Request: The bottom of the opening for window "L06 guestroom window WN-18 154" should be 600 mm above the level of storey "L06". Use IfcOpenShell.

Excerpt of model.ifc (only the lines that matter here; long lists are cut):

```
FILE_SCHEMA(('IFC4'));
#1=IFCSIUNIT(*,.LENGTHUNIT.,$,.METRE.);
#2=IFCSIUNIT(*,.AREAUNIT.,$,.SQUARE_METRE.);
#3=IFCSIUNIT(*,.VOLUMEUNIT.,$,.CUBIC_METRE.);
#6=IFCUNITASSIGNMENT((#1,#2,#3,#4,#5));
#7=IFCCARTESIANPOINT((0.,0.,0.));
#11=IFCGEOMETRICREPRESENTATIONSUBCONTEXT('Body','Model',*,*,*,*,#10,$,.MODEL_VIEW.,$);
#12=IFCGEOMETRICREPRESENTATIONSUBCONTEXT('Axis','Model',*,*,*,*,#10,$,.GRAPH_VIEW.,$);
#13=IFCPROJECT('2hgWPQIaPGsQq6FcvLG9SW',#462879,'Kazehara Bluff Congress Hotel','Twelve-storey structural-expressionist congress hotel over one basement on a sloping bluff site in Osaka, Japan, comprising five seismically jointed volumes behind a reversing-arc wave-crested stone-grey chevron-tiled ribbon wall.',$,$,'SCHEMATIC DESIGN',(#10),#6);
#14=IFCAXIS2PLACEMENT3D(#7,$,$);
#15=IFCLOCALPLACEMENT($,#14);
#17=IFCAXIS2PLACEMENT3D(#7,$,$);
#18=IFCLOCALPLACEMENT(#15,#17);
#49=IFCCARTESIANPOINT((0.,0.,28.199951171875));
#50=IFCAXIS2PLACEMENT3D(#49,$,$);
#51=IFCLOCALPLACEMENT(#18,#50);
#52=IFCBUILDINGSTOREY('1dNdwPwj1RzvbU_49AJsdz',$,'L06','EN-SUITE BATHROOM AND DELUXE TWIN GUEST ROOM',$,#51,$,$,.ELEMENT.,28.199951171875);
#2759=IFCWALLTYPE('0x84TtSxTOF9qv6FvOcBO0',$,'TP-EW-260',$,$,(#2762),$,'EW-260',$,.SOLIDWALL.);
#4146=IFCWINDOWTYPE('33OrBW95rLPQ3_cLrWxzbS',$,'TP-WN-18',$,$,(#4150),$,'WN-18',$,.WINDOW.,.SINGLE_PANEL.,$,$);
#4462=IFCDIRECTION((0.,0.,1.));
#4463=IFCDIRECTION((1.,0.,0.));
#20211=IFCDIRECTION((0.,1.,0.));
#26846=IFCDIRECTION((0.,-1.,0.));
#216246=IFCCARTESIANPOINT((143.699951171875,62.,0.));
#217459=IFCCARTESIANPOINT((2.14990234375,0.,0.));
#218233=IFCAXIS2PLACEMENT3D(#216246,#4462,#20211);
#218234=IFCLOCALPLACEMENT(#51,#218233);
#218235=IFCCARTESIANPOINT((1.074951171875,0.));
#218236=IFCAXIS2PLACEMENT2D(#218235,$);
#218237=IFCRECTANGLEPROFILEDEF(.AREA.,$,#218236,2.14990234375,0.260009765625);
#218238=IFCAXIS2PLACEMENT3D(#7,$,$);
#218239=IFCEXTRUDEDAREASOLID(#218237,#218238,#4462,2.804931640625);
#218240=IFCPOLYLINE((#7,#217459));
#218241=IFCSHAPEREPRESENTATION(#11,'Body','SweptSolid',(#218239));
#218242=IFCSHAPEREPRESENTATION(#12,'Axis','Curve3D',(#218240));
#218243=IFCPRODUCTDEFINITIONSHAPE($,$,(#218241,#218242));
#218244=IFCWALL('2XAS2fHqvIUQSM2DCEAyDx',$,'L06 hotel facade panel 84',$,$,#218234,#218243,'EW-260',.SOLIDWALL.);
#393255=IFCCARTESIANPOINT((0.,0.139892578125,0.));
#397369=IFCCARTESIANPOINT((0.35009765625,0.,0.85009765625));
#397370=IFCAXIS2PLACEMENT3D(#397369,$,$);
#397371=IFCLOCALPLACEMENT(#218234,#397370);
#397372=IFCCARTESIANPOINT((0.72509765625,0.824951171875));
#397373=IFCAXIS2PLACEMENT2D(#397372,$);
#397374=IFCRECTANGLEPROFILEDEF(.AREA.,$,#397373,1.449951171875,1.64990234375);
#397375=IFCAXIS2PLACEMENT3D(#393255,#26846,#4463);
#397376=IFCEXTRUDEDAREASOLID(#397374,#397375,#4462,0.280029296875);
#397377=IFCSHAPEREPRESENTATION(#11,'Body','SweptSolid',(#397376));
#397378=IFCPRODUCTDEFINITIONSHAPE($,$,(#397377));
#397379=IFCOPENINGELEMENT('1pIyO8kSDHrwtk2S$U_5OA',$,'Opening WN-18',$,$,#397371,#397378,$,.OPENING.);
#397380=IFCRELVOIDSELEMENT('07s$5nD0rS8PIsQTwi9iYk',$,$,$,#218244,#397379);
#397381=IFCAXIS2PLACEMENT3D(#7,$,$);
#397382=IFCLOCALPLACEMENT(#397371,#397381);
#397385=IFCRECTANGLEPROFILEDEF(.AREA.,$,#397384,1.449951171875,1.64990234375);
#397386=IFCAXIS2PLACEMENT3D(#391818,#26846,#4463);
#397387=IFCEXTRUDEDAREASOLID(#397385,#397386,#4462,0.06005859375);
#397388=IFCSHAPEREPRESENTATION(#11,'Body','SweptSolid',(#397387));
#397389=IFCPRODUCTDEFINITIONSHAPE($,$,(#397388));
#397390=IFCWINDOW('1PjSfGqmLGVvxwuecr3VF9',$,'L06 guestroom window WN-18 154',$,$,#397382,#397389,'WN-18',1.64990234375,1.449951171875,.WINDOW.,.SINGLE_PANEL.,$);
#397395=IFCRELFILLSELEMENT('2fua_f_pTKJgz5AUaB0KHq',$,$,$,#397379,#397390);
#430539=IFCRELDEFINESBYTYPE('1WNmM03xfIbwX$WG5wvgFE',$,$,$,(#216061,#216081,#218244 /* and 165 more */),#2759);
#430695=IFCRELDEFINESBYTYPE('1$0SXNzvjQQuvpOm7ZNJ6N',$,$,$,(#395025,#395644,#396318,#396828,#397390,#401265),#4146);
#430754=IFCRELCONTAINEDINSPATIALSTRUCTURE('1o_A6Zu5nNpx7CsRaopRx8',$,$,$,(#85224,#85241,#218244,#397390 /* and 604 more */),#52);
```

```python
import numpy as np
import ifcopenshell
import ifcopenshell.api.geometry
import ifcopenshell.geom
import ifcopenshell.util.element
import ifcopenshell.util.placement
import ifcopenshell.util.shape
import ifcopenshell.util.unit

model = ifcopenshell.open("model.ifc")
unit_scale = ifcopenshell.util.unit.calculate_unit_scale(model)

window = model.by_guid("1PjSfGqmLGVvxwuecr3VF9")
opening = window.FillsVoids[0].RelatingOpeningElement
storey = ifcopenshell.util.element.get_container(window, ifc_class="IfcBuildingStorey")
level = ifcopenshell.util.placement.get_local_placement(storey.ObjectPlacement)[2, 3]

# The opening's origin need not be at the sill, so measure its lowest point.
shape = ifcopenshell.geom.create_shape(ifcopenshell.geom.settings(), opening)
bottom = ifcopenshell.util.shape.get_shape_bottom_elevation(shape, shape.geometry) / unit_scale
dz = level + 0.6 / unit_scale - bottom

shift = np.array([0.0, 0.0, dz])
# The window is placed relative to its opening, so it follows when the opening moves.
matrix = ifcopenshell.util.placement.get_local_placement(opening.ObjectPlacement)
matrix[:3, 3] += shift
ifcopenshell.api.geometry.edit_object_placement(
    model, product=opening, matrix=matrix, is_si=False, should_transform_children=True
)

print(f"moved by {dz * unit_scale:+.3f} m")

model.write("model_updated.ifc")
```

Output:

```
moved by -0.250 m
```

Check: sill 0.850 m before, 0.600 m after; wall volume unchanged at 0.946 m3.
